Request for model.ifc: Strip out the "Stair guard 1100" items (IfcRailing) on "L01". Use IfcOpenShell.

First a look at what the model holds.

```python
import ifcopenshell
import ifcopenshell.util.element

model = ifcopenshell.open("model.ifc")
print(model.schema)
storey = next(s for s in model.by_type("IfcBuildingStorey") if s.Name == "L01")
railings = [e for e in ifcopenshell.util.element.get_decomposition(storey) if e.is_a("IfcRailing")]
seen = {}
for e in railings:
    element_type = ifcopenshell.util.element.get_type(e)
    name = element_type.Name if element_type not in (None, e) else None
    seen[name] = seen.get(name, 0) + 1
for name, count in sorted(seen.items(), key=str):
    print(count, "x", name)
```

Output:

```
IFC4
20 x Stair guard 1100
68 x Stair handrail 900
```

```python
import ifcopenshell
import ifcopenshell.api.root
import ifcopenshell.util.element

model = ifcopenshell.open("model.ifc")

storey = next(s for s in model.by_type("IfcBuildingStorey") if s.Name == "L01")
railings = [e for e in ifcopenshell.util.element.get_decomposition(storey) if e.is_a("IfcRailing")]
targets = [e for e in railings if (t := ifcopenshell.util.element.get_type(e)) not in (None, e) and t.Name == "Stair guard 1100"]

for e in targets:
    ifcopenshell.api.root.remove_product(model, product=e)
print(len(targets), "removed")

model.write("model_updated.ifc")
```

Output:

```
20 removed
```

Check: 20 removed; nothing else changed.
